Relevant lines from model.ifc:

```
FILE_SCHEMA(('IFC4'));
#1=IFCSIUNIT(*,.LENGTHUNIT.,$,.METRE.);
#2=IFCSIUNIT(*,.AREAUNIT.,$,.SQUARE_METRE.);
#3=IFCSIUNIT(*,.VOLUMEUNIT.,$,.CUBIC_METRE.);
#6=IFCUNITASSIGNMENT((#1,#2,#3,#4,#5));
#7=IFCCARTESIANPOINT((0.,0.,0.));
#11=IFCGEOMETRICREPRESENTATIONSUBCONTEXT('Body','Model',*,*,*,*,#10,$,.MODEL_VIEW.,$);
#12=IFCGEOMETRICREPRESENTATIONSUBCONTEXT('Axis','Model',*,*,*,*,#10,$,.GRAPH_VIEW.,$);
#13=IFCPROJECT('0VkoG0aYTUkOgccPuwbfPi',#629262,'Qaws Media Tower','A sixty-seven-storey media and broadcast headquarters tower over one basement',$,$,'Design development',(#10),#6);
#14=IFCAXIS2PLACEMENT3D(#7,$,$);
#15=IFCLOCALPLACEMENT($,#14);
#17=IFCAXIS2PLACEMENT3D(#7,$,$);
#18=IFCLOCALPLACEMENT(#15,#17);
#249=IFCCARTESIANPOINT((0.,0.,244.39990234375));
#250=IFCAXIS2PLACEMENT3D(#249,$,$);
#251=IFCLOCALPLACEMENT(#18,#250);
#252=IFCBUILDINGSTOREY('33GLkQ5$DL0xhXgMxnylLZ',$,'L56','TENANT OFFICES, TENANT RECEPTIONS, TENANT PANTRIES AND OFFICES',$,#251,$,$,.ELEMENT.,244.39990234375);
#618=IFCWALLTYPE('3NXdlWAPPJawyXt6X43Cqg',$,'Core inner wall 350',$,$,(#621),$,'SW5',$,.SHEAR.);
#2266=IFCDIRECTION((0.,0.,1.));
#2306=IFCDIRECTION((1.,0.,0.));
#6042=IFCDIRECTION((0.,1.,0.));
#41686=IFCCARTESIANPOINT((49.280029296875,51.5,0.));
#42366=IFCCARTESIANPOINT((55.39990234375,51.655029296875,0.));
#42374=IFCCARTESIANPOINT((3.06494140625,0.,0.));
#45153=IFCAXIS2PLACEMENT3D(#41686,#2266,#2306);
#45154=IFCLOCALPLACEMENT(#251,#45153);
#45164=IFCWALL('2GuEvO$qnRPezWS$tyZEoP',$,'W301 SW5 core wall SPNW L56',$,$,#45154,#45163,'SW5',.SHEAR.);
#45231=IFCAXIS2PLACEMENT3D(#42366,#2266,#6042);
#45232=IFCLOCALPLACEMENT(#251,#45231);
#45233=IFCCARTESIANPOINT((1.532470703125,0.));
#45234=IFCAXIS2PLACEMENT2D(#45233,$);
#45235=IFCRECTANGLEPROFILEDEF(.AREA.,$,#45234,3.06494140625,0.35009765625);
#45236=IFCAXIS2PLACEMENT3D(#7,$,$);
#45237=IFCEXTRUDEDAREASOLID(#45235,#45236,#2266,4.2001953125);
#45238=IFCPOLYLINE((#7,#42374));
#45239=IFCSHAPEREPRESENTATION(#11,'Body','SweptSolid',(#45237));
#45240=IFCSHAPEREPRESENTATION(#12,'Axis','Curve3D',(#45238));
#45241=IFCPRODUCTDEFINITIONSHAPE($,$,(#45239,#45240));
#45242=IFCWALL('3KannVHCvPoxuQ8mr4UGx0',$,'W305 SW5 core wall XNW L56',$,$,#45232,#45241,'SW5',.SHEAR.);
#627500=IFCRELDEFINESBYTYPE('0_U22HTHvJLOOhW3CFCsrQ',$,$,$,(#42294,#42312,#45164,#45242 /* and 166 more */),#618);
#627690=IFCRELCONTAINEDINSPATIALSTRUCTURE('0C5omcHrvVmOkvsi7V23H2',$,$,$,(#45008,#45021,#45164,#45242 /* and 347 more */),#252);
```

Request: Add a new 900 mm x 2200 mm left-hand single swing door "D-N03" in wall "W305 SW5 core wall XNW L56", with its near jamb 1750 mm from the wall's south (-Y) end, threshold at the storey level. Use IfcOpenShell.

```python
import numpy as np
import ifcopenshell
import ifcopenshell.api.feature
import ifcopenshell.api.geometry
import ifcopenshell.api.root
import ifcopenshell.api.spatial
import ifcopenshell.geom
import ifcopenshell.util.element
import ifcopenshell.util.placement
import ifcopenshell.util.representation
import ifcopenshell.util.shape
import ifcopenshell.util.unit

model = ifcopenshell.open("model.ifc")
unit_scale = ifcopenshell.util.unit.calculate_unit_scale(model)
settings = ifcopenshell.geom.settings()


def volume(element):
    """Net volume in cubic metres, openings subtracted."""
    shape = ifcopenshell.geom.create_shape(settings, element)
    return ifcopenshell.util.shape.get_volume(shape.geometry)


wall = model.by_id(45242)
storey = ifcopenshell.util.element.get_container(wall, ifc_class="IfcBuildingStorey")
context = ifcopenshell.util.representation.get_context(model, "Model", "Body", "MODEL_VIEW")
before = volume(wall)

width, height, from_end, sill = 0.9, 2.2, 1.75, 0.0  # metres

# The wall runs along its own X axis, and the end named is its -X end.
wall_shape = ifcopenshell.geom.create_shape(settings, wall)
x, y, z = ifcopenshell.util.shape.get_vertices(wall_shape.geometry).T
start = x.min() + from_end
face, thickness = float(y.min()), float(y.max() - y.min())
wall_matrix = ifcopenshell.util.placement.get_local_placement(wall.ObjectPlacement)
level = ifcopenshell.util.placement.get_local_placement(storey.ObjectPlacement)[2, 3]


def in_wall(x, y):
    """Placement at x, y metres in the wall's axes, at sill height."""
    matrix = wall_matrix.copy()
    matrix[:, 3] = wall_matrix @ np.array([x / unit_scale, y / unit_scale, 0.0, 1.0])
    matrix[2, 3] = level + sill / unit_scale
    return matrix


# Opening: a box that overshoots both wall faces by 50 mm.
opening = ifcopenshell.api.root.create_entity(model, ifc_class="IfcOpeningElement", predefined_type="OPENING")
box = ifcopenshell.api.geometry.add_wall_representation(
    model, context=context, length=width, height=height, thickness=thickness + 0.1
)
ifcopenshell.api.geometry.assign_representation(model, product=opening, representation=box)
ifcopenshell.api.geometry.edit_object_placement(model, product=opening, matrix=in_wall(start, face - 0.05), is_si=False)
ifcopenshell.api.feature.add_feature(model, feature=opening, element=wall)

door = ifcopenshell.api.root.create_entity(model, ifc_class="IfcDoor", name="D-N03", predefined_type="DOOR")
door.OverallWidth, door.OverallHeight = width / unit_scale, height / unit_scale
door.OperationType = "SINGLE_SWING_LEFT"
body = ifcopenshell.api.geometry.add_door_representation(
    model,
    context=context,
    overall_width=door.OverallWidth,
    overall_height=door.OverallHeight,
    operation_type="SINGLE_SWING_LEFT",
    lining_properties={"LiningDepth": thickness / unit_scale, "ThresholdDepth": thickness / unit_scale},
)
ifcopenshell.api.geometry.assign_representation(model, product=door, representation=body)
ifcopenshell.api.spatial.assign_container(model, products=[door], relating_structure=storey)
ifcopenshell.api.feature.add_filling(model, opening=opening, element=door)

# The lining spans the wall, so the door starts at the wall face.
ifcopenshell.api.geometry.edit_object_placement(model, product=door, matrix=in_wall(start, face), is_si=False)

after = volume(wall)

print(f"wall volume {before:.3f} -> {after:.3f} m3")

model.write("model_edited.ifc")
```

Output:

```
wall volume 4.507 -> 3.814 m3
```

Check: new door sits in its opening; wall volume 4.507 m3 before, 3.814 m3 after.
